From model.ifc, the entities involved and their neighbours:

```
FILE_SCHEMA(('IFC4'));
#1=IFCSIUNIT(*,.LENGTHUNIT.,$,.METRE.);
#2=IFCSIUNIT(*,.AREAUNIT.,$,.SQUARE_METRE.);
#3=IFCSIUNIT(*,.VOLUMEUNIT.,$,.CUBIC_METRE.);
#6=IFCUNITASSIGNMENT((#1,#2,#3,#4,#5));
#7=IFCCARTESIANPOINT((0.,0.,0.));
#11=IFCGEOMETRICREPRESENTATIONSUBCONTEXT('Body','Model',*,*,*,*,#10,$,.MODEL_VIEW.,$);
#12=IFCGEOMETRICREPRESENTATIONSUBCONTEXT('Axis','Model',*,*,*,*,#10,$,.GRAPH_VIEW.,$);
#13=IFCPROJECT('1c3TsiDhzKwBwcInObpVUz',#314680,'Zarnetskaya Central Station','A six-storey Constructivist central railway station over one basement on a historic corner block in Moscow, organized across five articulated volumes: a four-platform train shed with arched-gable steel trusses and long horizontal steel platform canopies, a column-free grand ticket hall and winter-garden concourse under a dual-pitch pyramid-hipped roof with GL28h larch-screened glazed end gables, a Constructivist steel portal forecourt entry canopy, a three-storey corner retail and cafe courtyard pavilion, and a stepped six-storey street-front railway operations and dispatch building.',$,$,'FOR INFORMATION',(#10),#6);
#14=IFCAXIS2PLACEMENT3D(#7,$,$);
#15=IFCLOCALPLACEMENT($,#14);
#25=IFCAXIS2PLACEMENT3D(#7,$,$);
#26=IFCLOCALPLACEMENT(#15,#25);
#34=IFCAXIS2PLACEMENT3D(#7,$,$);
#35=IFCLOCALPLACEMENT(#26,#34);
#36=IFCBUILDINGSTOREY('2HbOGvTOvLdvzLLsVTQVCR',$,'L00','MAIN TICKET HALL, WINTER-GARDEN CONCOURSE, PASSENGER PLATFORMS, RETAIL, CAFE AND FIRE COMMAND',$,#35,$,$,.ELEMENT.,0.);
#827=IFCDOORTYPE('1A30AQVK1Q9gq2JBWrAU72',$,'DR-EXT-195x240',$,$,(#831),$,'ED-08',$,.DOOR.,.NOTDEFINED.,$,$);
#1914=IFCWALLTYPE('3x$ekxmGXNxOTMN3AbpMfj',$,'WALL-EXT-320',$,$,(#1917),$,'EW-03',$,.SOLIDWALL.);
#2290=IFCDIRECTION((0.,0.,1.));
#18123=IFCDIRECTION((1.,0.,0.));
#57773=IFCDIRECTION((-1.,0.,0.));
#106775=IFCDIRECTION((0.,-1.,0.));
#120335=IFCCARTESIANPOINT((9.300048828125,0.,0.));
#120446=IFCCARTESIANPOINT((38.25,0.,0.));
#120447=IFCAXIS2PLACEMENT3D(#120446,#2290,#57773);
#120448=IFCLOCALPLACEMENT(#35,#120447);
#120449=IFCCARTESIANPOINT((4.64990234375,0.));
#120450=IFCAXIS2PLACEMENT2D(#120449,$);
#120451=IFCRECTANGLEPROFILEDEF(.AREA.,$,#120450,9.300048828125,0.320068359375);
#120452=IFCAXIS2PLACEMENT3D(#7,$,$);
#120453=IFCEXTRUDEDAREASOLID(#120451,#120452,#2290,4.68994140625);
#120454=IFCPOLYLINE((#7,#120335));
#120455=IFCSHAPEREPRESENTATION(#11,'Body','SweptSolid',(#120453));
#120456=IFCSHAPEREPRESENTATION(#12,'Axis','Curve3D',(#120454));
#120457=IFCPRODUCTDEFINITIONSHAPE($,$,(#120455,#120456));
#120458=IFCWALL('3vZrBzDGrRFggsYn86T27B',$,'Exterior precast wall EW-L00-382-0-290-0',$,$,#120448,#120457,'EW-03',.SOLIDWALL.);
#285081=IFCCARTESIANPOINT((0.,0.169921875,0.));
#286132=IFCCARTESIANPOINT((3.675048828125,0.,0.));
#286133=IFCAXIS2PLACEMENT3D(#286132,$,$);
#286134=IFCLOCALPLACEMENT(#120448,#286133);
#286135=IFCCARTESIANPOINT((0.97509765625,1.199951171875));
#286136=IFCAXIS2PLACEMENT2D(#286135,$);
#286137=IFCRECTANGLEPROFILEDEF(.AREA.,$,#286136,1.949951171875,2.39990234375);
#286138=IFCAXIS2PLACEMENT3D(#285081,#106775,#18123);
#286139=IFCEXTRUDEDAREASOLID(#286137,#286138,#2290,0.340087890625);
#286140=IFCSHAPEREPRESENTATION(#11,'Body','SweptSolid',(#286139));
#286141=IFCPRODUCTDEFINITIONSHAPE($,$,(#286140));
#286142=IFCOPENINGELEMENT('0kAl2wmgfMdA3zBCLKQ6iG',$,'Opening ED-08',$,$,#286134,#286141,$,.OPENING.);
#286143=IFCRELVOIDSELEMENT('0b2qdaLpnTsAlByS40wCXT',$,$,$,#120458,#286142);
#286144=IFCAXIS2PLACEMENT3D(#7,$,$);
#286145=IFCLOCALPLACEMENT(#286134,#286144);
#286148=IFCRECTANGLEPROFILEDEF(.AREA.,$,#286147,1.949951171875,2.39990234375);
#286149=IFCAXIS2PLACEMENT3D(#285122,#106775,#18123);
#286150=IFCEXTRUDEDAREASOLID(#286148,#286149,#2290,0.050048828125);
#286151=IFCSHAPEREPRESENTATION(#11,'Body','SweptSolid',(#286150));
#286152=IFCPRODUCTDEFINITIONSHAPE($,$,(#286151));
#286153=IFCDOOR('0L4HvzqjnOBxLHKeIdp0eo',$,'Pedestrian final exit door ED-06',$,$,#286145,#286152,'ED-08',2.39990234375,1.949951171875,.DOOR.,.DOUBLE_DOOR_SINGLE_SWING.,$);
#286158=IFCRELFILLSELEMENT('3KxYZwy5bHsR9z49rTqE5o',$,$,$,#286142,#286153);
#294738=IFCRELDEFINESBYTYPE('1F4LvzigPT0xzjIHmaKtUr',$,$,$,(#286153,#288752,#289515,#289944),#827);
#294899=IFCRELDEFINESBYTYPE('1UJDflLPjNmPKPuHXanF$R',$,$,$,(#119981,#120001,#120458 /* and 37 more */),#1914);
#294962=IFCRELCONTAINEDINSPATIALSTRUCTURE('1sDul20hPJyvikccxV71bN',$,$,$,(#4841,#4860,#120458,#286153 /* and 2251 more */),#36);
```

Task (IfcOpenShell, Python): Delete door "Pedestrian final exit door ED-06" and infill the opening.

```python
import ifcopenshell
import ifcopenshell.api.feature
import ifcopenshell.api.root
import ifcopenshell.geom
import ifcopenshell.util.shape

model = ifcopenshell.open("model.ifc")
settings = ifcopenshell.geom.settings()


def volume(element):
    """Net volume in cubic metres, openings subtracted."""
    shape = ifcopenshell.geom.create_shape(settings, element)
    return ifcopenshell.util.shape.get_volume(shape.geometry)


door = model.by_id(286153)
opening = door.FillsVoids[0].RelatingOpeningElement
wall = opening.VoidsElements[0].RelatingBuildingElement
before = volume(wall)

ifcopenshell.api.root.remove_product(model, product=door)
ifcopenshell.api.feature.remove_feature(model, feature=opening)

after = volume(wall)

print(f"wall volume {before:.3f} -> {after:.3f} m3")

model.write("model_rev.ifc")
```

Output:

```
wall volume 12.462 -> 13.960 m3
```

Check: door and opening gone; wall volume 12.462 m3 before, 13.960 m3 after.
